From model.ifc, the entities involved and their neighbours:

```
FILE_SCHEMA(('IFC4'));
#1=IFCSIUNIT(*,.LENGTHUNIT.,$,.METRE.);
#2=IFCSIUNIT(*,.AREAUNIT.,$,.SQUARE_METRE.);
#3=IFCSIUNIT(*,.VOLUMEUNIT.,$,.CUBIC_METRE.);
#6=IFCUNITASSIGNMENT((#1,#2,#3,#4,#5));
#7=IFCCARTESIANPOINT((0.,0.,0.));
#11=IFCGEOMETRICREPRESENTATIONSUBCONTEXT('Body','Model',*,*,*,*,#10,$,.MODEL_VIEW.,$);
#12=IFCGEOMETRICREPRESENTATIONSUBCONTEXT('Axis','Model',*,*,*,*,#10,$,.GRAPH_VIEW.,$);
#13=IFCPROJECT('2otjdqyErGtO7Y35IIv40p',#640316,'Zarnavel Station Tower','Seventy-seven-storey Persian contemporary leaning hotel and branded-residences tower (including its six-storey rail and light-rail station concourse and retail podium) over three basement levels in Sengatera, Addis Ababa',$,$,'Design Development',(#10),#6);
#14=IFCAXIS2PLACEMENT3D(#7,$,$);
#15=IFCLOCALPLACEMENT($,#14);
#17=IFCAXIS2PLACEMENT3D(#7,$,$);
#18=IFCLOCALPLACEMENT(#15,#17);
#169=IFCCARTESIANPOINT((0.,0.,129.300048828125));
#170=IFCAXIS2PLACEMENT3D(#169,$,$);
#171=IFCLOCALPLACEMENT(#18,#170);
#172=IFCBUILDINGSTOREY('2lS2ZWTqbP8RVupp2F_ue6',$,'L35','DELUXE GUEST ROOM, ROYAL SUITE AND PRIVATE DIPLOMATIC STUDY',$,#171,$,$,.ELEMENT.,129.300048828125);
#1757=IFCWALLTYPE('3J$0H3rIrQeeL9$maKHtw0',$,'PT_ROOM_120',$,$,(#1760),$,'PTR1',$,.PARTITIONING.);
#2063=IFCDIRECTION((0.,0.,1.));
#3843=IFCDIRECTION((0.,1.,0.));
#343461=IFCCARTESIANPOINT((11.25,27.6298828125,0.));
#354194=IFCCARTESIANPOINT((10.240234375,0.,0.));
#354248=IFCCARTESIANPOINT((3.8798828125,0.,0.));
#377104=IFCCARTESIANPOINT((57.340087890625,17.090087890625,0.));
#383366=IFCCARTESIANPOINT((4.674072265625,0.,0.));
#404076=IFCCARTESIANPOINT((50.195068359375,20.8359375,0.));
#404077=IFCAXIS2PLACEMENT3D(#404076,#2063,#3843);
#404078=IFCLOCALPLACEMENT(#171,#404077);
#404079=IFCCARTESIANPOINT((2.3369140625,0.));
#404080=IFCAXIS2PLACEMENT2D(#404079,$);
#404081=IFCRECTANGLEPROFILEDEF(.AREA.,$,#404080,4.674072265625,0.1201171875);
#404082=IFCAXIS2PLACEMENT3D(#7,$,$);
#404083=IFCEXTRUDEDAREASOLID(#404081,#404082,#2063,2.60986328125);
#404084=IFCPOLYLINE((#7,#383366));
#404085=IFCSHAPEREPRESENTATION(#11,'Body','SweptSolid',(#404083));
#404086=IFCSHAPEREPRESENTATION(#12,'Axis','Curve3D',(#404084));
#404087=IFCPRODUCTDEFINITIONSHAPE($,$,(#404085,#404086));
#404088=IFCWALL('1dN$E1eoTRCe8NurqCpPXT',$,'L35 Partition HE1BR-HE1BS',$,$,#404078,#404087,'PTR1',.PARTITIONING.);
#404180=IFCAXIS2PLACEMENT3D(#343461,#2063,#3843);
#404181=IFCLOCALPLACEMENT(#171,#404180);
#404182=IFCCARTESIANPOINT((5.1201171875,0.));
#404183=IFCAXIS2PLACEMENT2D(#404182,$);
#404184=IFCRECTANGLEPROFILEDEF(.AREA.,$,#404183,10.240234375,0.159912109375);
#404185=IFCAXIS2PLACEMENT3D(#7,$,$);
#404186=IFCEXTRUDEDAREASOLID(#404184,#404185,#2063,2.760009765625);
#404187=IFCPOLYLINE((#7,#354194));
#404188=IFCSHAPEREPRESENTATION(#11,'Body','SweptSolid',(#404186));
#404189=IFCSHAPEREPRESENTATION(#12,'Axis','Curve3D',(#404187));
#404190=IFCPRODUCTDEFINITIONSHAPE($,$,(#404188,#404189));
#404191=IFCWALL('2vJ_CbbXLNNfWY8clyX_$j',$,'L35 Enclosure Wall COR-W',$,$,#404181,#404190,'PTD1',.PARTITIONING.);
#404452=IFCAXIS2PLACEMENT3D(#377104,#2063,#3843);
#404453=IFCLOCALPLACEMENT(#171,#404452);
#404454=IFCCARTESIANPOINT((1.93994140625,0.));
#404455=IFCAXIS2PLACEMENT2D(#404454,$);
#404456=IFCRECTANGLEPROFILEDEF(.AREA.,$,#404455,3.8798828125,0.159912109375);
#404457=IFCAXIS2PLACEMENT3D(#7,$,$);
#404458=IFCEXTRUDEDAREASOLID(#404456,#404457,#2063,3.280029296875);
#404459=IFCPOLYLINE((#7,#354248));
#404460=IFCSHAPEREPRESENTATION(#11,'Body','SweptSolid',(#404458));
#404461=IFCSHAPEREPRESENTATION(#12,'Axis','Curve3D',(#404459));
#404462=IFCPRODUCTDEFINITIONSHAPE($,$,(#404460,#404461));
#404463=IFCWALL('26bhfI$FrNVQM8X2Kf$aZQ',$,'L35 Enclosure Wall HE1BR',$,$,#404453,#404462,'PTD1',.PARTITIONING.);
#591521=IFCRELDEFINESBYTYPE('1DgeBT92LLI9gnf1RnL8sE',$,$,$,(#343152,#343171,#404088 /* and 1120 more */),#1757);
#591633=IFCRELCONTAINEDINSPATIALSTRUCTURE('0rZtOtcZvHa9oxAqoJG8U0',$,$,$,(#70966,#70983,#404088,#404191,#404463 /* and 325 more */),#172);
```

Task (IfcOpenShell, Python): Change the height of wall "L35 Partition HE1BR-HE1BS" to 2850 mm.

```python
import ifcopenshell
import ifcopenshell.geom
import ifcopenshell.util.representation
import ifcopenshell.util.shape

model = ifcopenshell.open("model.ifc")
settings = ifcopenshell.geom.settings()


def volume(element):
    """Net volume in cubic metres, openings subtracted."""
    shape = ifcopenshell.geom.create_shape(settings, element)
    return ifcopenshell.util.shape.get_volume(shape.geometry)


wall = model.by_guid("1dN$E1eoTRCe8NurqCpPXT")
before = volume(wall)

body = ifcopenshell.util.representation.get_representation(wall, "Model", "Body")
solid = body.Items[0]
old_height = solid.Depth
solid.Depth = 2.85
after = volume(wall)

print(f"height {old_height:g} -> {solid.Depth:g}, volume {before:.3f} -> {after:.3f} m3")

model.write("model_v2.ifc")
```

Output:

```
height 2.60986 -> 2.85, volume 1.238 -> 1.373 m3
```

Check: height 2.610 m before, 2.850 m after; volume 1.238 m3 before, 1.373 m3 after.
